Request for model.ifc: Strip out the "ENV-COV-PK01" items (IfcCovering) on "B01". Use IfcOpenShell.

First a look at what the model holds.

```python
import ifcopenshell
import ifcopenshell.util.element

model = ifcopenshell.open("model.ifc")
print(model.schema)
storey = next(s for s in model.by_type("IfcBuildingStorey") if s.Name == "B01")
coverings = [e for e in ifcopenshell.util.element.get_decomposition(storey) if e.is_a("IfcCovering")]
seen = {}
for e in coverings:
    element_type = ifcopenshell.util.element.get_type(e)
    name = element_type.Name if element_type not in (None, e) else None
    seen[name] = seen.get(name, 0) + 1
for name, count in sorted(seen.items(), key=str):
    print(count, "x", name)
```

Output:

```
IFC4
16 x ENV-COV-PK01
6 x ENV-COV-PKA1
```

```python
import ifcopenshell
import ifcopenshell.api.root
import ifcopenshell.util.element

model = ifcopenshell.open("model.ifc")

storey = next(s for s in model.by_type("IfcBuildingStorey") if s.Name == "B01")
coverings = [e for e in ifcopenshell.util.element.get_decomposition(storey) if e.is_a("IfcCovering")]
targets = [e for e in coverings if (t := ifcopenshell.util.element.get_type(e)) not in (None, e) and t.Name == "ENV-COV-PK01"]

for e in targets:
    ifcopenshell.api.root.remove_product(model, product=e)
print(len(targets), "removed")

model.write("model_v2.ifc")
```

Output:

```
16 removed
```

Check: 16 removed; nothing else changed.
